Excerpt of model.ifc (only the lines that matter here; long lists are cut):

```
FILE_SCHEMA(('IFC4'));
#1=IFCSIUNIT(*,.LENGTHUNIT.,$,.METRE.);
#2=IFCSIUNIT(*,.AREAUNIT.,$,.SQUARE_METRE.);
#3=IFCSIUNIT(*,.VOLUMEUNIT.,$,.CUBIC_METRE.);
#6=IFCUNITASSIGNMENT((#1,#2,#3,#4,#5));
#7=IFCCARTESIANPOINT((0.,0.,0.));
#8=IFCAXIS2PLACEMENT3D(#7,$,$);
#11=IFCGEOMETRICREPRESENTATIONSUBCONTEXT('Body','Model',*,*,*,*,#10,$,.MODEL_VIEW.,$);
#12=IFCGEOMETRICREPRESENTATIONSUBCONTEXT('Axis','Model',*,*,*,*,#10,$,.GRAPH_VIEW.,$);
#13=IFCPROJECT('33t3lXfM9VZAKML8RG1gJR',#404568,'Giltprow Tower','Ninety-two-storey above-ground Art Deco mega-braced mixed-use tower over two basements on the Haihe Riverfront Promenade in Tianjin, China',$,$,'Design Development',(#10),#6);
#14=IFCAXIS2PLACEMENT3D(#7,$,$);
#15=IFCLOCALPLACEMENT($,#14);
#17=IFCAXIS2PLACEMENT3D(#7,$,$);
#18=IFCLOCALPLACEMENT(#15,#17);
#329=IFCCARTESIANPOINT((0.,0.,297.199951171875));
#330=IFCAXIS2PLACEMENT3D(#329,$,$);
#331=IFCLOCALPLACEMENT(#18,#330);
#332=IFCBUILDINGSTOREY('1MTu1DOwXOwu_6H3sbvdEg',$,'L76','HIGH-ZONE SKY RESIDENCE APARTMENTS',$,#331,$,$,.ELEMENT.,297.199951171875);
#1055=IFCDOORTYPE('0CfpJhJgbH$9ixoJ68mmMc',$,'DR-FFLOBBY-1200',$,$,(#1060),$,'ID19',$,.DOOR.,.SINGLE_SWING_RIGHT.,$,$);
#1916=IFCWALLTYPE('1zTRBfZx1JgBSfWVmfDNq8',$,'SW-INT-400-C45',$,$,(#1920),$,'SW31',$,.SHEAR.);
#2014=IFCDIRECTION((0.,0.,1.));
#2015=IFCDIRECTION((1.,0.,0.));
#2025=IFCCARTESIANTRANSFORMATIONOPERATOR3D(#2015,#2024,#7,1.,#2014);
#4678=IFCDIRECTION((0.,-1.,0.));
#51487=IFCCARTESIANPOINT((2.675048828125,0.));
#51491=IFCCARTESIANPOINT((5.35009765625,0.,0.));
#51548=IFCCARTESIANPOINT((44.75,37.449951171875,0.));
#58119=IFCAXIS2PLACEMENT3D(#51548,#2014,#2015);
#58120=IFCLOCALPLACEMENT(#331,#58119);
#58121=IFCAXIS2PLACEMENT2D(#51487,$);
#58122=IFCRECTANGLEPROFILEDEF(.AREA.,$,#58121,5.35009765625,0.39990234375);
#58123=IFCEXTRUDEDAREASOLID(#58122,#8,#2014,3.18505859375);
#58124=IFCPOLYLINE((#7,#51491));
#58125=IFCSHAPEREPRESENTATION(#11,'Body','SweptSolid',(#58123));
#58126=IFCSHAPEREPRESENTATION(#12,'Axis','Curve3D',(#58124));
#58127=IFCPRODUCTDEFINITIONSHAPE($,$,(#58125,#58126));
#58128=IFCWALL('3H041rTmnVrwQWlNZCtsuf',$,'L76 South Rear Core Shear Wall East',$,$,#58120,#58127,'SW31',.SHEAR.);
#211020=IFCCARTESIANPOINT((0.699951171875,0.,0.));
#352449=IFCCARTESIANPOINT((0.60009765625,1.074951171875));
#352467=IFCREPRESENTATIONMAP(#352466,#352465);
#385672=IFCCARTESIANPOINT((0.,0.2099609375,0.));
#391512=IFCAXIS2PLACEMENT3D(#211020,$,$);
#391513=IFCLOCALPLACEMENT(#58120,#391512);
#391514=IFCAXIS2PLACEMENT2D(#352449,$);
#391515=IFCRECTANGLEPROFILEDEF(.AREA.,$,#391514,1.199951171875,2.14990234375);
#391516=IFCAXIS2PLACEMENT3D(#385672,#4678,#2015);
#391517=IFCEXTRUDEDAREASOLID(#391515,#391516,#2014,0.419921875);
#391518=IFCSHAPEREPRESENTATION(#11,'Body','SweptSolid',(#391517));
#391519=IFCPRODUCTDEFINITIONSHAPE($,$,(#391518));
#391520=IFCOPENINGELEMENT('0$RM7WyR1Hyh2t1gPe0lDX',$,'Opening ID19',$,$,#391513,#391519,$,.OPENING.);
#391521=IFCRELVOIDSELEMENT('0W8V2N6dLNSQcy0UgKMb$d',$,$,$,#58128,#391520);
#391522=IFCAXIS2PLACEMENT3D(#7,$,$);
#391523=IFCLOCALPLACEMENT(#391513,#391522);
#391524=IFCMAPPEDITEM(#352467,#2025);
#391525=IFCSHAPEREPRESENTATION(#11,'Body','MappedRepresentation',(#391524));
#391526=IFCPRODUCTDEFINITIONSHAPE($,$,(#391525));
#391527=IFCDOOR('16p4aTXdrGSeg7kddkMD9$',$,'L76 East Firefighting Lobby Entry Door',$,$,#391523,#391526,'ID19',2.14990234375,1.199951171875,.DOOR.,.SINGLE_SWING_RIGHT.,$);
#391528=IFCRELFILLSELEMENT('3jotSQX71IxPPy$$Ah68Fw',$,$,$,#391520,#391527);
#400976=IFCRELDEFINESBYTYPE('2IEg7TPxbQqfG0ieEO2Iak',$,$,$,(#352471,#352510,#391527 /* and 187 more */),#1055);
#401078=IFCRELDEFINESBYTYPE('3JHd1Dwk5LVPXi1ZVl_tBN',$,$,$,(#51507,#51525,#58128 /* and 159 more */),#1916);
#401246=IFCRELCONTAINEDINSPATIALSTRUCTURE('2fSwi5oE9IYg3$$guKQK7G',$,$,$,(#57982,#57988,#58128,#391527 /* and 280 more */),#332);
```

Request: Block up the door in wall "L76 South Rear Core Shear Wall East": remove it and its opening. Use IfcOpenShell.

```python
import ifcopenshell
import ifcopenshell.api.feature
import ifcopenshell.api.root
import ifcopenshell.geom
import ifcopenshell.util.shape

model = ifcopenshell.open("model.ifc")
settings = ifcopenshell.geom.settings()


def volume(element):
    """Net volume in cubic metres, openings subtracted."""
    shape = ifcopenshell.geom.create_shape(settings, element)
    return ifcopenshell.util.shape.get_volume(shape.geometry)


door = model.by_guid("16p4aTXdrGSeg7kddkMD9$")
opening = door.FillsVoids[0].RelatingOpeningElement
wall = opening.VoidsElements[0].RelatingBuildingElement
before = volume(wall)

ifcopenshell.api.root.remove_product(model, product=door)
ifcopenshell.api.feature.remove_feature(model, feature=opening)

after = volume(wall)

print(f"wall volume {before:.3f} -> {after:.3f} m3")

model.write("model_v2.ifc")
```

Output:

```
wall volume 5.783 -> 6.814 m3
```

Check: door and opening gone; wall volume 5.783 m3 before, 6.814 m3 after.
